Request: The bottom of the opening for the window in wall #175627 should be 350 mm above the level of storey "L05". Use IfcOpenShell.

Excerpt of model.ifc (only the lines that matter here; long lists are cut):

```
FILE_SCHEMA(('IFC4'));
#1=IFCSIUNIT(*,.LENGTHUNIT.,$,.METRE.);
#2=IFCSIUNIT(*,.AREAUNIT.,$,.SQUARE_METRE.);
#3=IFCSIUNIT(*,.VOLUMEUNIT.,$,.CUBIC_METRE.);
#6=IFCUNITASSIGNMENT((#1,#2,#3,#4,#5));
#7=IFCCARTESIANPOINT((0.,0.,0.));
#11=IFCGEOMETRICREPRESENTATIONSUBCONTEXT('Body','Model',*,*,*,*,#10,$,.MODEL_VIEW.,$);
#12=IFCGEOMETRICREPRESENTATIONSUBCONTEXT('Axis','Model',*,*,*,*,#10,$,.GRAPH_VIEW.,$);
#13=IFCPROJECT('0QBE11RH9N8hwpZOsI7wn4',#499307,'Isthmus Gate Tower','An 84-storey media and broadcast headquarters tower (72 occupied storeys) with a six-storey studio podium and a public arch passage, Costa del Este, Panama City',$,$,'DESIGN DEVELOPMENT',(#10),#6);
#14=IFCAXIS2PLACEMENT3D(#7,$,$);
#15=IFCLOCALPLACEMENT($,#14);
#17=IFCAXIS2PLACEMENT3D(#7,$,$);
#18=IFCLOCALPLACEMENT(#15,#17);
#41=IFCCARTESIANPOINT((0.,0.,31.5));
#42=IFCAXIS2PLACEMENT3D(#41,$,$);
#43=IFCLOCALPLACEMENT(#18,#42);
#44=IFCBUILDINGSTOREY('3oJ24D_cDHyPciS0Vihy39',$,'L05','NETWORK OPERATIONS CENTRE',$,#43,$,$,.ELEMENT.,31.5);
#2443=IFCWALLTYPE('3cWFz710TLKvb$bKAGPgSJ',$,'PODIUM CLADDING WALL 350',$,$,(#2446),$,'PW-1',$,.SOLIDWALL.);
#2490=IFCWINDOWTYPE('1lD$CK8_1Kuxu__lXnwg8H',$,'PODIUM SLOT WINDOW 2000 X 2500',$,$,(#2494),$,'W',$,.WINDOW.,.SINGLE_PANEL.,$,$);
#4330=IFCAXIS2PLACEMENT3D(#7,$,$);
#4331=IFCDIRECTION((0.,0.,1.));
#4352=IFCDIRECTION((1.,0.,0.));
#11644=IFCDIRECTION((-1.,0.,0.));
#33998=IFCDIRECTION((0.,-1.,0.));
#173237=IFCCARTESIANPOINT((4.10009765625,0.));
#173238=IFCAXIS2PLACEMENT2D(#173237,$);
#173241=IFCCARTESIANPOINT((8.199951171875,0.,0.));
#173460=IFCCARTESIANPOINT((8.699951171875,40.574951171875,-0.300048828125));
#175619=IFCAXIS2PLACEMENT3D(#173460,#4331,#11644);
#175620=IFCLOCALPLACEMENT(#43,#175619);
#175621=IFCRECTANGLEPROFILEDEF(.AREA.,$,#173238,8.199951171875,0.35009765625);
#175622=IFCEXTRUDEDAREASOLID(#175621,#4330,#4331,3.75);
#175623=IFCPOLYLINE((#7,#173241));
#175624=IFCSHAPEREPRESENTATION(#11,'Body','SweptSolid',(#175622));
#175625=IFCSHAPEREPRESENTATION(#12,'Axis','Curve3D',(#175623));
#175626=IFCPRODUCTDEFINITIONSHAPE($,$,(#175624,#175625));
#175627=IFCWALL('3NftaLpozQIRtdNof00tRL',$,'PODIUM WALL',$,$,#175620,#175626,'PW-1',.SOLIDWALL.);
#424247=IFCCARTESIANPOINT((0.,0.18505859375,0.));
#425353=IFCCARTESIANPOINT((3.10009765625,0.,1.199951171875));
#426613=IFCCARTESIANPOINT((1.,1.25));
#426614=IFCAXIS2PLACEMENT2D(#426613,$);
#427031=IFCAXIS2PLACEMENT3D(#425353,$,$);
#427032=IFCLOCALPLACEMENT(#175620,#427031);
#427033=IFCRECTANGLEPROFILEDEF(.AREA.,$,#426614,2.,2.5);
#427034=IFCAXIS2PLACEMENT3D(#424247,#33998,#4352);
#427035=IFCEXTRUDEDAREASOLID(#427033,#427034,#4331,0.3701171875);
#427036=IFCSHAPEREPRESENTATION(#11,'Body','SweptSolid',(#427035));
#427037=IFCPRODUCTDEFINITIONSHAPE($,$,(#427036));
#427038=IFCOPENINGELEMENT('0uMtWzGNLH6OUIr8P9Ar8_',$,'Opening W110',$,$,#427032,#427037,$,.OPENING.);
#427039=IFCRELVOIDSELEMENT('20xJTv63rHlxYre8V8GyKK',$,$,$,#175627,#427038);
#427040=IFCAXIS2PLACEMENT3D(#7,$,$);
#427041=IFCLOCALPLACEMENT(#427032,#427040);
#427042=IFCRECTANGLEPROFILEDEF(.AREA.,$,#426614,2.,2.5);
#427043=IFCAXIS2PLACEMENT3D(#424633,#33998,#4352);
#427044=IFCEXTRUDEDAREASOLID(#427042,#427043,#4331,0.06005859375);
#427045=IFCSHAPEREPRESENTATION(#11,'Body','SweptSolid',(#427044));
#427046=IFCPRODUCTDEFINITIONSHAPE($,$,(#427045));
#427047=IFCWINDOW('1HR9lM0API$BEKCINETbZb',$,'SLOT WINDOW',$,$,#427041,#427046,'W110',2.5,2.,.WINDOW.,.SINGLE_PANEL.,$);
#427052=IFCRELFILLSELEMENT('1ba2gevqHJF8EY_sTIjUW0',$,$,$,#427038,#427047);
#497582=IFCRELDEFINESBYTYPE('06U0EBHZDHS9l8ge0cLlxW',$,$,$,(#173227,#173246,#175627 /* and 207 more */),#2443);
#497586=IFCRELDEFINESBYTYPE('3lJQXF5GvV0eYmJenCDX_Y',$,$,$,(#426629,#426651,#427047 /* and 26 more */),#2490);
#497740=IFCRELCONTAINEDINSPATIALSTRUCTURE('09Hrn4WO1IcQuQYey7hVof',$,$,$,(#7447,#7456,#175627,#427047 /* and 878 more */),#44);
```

```python
import numpy as np
import ifcopenshell
import ifcopenshell.api.geometry
import ifcopenshell.geom
import ifcopenshell.util.element
import ifcopenshell.util.placement
import ifcopenshell.util.shape
import ifcopenshell.util.unit

model = ifcopenshell.open("model.ifc")
unit_scale = ifcopenshell.util.unit.calculate_unit_scale(model)

window = model.by_guid("1HR9lM0API$BEKCINETbZb")
opening = window.FillsVoids[0].RelatingOpeningElement
storey = ifcopenshell.util.element.get_container(window, ifc_class="IfcBuildingStorey")
level = ifcopenshell.util.placement.get_local_placement(storey.ObjectPlacement)[2, 3]

# The opening's origin need not be at the sill, so measure its lowest point.
shape = ifcopenshell.geom.create_shape(ifcopenshell.geom.settings(), opening)
bottom = ifcopenshell.util.shape.get_shape_bottom_elevation(shape, shape.geometry) / unit_scale
dz = level + 0.35 - bottom

shift = np.array([0.0, 0.0, dz])
# The window is placed relative to its opening, so it follows when the opening moves.
matrix = ifcopenshell.util.placement.get_local_placement(opening.ObjectPlacement)
matrix[:3, 3] += shift
ifcopenshell.api.geometry.edit_object_placement(
    model, product=opening, matrix=matrix, is_si=False, should_transform_children=True
)

print(f"moved by {dz * unit_scale:+.3f} m")

model.write("model-out.ifc")
```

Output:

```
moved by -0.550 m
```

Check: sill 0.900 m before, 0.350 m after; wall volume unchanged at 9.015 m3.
